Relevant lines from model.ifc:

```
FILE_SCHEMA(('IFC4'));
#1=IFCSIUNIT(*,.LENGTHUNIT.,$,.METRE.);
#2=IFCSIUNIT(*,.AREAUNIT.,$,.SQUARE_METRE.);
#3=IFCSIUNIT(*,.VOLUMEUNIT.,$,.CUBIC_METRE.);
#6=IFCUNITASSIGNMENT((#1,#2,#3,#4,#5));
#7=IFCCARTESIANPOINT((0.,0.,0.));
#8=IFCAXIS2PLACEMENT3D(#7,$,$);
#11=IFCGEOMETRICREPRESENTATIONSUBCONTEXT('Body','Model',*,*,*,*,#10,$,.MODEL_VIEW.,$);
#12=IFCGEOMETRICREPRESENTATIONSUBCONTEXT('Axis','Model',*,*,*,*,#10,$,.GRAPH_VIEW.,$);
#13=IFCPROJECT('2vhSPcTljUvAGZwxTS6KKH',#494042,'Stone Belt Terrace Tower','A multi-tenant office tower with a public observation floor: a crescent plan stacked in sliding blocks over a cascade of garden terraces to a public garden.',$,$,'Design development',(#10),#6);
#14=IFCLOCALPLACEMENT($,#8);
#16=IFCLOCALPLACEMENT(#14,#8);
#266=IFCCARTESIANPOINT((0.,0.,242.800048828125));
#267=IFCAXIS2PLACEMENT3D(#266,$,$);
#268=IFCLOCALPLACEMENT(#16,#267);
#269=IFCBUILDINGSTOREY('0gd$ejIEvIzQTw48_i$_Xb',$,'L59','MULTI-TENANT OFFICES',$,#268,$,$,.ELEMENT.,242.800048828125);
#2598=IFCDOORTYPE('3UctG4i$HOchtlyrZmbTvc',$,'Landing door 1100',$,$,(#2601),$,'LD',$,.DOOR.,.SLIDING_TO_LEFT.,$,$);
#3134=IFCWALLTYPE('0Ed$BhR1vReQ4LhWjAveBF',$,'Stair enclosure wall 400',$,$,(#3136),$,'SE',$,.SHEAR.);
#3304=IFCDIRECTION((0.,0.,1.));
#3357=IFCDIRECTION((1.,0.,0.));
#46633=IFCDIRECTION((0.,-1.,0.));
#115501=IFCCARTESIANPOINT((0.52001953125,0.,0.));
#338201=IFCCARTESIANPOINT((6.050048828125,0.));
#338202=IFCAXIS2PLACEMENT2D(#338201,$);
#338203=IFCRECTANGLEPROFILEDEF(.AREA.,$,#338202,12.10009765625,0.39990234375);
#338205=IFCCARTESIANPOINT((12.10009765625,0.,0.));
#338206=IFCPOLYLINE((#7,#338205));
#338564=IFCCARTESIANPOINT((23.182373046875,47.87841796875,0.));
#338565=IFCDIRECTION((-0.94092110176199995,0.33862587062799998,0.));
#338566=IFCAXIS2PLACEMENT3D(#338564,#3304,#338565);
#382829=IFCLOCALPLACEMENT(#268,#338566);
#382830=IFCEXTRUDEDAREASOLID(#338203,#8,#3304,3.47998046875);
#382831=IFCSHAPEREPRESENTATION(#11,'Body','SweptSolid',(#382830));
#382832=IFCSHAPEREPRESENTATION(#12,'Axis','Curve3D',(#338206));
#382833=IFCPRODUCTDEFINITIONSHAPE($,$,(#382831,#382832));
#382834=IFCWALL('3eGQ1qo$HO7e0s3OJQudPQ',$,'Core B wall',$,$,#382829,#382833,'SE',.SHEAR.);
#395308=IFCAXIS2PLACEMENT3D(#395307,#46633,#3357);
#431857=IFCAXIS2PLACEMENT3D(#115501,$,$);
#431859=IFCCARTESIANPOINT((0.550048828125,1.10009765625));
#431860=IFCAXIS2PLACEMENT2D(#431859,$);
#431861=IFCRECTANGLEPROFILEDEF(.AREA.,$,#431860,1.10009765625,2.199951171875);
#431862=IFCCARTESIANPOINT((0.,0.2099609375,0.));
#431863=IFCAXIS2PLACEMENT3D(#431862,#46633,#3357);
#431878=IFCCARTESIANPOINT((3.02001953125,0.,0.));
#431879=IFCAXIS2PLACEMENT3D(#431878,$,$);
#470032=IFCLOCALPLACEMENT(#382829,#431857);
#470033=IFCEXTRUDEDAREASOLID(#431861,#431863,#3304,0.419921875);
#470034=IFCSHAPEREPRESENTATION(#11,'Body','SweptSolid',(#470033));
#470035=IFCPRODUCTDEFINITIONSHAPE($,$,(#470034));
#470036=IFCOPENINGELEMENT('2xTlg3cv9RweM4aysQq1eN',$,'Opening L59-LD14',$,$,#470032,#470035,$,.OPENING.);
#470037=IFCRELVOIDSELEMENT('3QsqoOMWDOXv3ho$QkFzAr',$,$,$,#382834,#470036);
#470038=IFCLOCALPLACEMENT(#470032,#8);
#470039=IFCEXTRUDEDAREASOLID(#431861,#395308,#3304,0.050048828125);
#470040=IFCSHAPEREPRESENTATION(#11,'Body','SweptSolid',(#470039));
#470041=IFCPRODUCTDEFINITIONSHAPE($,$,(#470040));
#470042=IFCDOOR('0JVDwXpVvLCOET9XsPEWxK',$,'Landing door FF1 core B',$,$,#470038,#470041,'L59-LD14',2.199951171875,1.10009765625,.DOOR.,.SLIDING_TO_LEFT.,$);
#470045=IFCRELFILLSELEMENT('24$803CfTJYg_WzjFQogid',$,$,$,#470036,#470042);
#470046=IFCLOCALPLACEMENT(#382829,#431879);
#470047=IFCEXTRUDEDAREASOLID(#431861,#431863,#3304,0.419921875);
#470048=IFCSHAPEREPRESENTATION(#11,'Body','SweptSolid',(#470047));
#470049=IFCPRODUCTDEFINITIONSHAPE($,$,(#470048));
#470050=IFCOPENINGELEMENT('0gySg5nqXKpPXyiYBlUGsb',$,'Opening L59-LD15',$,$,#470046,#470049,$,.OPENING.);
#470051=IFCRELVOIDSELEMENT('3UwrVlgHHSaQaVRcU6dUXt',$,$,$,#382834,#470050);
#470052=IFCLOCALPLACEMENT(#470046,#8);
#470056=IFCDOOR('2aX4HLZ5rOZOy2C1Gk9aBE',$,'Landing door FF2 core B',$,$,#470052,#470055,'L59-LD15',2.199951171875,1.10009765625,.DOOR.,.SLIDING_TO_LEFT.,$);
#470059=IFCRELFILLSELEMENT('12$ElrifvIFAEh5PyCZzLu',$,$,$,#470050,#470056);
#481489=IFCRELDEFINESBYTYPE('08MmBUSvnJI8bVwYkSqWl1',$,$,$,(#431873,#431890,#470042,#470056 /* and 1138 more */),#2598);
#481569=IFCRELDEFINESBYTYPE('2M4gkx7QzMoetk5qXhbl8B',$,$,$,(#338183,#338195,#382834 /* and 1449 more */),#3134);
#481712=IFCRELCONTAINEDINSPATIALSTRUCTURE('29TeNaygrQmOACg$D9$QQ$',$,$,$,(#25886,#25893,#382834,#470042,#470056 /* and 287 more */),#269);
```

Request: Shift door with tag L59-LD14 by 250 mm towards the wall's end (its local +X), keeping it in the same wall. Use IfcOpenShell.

```python
import ifcopenshell
import ifcopenshell.api.geometry
import ifcopenshell.util.placement
import ifcopenshell.util.unit

model = ifcopenshell.open("model.ifc")
unit_scale = ifcopenshell.util.unit.calculate_unit_scale(model)

door = model.by_id(470042)
opening = door.FillsVoids[0].RelatingOpeningElement
wall = opening.VoidsElements[0].RelatingBuildingElement

wall_matrix = ifcopenshell.util.placement.get_local_placement(wall.ObjectPlacement)
shift = wall_matrix[:3, 0] * 0.25 / unit_scale
before = ifcopenshell.util.placement.get_local_placement(door.ObjectPlacement)[:3, 3].copy()

# The door is placed relative to its opening, so it follows when the opening moves.
matrix = ifcopenshell.util.placement.get_local_placement(opening.ObjectPlacement)
matrix[:3, 3] += shift
ifcopenshell.api.geometry.edit_object_placement(
    model, product=opening, matrix=matrix, is_si=False, should_transform_children=True
)

after = ifcopenshell.util.placement.get_local_placement(door.ObjectPlacement)[:3, 3]
print("door moved by", (after - before).round(3) + 0.0)

model.write("model_updated.ifc")
```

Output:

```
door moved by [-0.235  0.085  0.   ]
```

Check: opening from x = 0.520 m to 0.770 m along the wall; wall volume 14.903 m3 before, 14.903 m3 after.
